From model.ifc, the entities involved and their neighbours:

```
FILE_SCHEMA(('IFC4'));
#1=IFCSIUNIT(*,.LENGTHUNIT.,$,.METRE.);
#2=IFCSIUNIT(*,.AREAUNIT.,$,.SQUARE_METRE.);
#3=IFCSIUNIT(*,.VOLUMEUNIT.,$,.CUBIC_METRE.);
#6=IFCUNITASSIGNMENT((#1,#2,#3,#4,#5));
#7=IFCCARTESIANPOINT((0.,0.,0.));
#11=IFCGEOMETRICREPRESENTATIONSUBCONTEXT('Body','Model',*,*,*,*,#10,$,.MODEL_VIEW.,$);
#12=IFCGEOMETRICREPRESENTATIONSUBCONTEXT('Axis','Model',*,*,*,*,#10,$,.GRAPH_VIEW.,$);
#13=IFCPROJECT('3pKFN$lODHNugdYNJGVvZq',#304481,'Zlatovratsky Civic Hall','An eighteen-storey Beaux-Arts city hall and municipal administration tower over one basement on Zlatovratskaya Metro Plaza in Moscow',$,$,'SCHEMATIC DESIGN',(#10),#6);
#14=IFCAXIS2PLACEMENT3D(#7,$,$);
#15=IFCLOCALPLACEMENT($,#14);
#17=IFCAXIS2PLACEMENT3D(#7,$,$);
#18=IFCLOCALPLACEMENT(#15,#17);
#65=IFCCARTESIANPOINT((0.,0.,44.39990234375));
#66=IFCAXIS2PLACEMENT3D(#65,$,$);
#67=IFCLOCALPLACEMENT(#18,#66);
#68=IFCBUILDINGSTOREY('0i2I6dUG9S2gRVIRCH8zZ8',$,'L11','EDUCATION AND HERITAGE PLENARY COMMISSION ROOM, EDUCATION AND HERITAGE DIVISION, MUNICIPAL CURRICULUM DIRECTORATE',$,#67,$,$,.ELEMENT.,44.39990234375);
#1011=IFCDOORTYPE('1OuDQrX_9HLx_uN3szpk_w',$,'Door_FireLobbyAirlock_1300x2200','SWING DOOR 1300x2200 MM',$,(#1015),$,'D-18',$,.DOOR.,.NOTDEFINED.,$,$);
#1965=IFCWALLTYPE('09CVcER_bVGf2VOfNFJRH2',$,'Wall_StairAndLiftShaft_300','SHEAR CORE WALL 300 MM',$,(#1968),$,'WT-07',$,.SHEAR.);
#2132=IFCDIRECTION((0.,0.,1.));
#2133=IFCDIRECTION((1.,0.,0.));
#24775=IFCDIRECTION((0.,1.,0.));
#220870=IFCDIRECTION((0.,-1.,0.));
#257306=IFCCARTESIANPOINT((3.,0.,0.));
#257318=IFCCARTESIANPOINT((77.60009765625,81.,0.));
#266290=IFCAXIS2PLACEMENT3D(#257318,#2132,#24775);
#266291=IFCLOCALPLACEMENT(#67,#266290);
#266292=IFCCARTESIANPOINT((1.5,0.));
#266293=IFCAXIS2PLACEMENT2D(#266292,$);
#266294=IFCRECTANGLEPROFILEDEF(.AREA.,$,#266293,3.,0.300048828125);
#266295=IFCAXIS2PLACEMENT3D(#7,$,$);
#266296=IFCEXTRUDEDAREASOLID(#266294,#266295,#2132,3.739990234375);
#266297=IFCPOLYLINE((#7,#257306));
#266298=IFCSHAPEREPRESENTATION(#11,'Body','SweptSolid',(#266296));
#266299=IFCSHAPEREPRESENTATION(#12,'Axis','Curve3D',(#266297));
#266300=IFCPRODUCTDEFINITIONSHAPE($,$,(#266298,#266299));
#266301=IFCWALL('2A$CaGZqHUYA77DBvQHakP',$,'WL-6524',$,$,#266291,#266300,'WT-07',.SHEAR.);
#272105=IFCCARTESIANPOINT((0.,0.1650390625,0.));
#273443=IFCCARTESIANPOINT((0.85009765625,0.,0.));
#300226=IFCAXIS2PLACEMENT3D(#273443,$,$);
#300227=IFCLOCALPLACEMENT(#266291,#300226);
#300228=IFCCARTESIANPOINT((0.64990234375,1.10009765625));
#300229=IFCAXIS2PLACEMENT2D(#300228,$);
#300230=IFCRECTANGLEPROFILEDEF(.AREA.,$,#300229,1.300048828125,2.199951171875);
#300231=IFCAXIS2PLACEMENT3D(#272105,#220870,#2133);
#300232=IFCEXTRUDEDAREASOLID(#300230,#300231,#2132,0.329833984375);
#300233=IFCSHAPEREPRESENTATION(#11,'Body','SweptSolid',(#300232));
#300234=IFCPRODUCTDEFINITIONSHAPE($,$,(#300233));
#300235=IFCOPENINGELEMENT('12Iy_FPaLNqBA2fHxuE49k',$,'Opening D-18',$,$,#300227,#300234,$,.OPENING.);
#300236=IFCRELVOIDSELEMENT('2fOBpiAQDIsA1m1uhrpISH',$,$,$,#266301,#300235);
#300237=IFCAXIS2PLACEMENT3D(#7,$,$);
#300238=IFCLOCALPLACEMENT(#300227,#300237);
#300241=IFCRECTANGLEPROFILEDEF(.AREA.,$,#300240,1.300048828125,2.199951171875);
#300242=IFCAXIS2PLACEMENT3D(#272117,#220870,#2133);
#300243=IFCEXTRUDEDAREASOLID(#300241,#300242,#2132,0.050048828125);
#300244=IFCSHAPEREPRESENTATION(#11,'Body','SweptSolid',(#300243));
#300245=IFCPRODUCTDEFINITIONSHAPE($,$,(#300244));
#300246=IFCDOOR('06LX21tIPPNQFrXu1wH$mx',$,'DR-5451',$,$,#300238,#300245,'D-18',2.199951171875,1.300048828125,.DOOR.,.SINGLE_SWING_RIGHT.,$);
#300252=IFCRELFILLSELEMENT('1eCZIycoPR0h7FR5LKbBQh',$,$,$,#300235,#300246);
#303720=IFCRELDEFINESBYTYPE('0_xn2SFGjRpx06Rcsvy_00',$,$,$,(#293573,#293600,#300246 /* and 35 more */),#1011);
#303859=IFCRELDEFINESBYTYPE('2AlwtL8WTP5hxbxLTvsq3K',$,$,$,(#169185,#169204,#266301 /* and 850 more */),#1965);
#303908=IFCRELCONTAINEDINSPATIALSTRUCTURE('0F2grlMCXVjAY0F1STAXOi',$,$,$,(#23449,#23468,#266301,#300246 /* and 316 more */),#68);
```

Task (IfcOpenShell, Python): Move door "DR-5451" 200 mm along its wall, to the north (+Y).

```python
import ifcopenshell
import ifcopenshell.api.geometry
import ifcopenshell.util.placement
import ifcopenshell.util.unit

model = ifcopenshell.open("model.ifc")
unit_scale = ifcopenshell.util.unit.calculate_unit_scale(model)

door = model.by_guid("06LX21tIPPNQFrXu1wH$mx")
opening = door.FillsVoids[0].RelatingOpeningElement
wall = opening.VoidsElements[0].RelatingBuildingElement

wall_matrix = ifcopenshell.util.placement.get_local_placement(wall.ObjectPlacement)
shift = wall_matrix[:3, 0] * 0.2 / unit_scale
before = ifcopenshell.util.placement.get_local_placement(door.ObjectPlacement)[:3, 3].copy()

# The door is placed relative to its opening, so it follows when the opening moves.
matrix = ifcopenshell.util.placement.get_local_placement(opening.ObjectPlacement)
matrix[:3, 3] += shift
ifcopenshell.api.geometry.edit_object_placement(
    model, product=opening, matrix=matrix, is_si=False, should_transform_children=True
)

after = ifcopenshell.util.placement.get_local_placement(door.ObjectPlacement)[:3, 3]
print("door moved by", (after - before).round(3) + 0.0)

model.write("model_edited.ifc")
```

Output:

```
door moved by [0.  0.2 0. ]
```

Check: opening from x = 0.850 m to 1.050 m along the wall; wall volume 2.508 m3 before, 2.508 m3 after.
